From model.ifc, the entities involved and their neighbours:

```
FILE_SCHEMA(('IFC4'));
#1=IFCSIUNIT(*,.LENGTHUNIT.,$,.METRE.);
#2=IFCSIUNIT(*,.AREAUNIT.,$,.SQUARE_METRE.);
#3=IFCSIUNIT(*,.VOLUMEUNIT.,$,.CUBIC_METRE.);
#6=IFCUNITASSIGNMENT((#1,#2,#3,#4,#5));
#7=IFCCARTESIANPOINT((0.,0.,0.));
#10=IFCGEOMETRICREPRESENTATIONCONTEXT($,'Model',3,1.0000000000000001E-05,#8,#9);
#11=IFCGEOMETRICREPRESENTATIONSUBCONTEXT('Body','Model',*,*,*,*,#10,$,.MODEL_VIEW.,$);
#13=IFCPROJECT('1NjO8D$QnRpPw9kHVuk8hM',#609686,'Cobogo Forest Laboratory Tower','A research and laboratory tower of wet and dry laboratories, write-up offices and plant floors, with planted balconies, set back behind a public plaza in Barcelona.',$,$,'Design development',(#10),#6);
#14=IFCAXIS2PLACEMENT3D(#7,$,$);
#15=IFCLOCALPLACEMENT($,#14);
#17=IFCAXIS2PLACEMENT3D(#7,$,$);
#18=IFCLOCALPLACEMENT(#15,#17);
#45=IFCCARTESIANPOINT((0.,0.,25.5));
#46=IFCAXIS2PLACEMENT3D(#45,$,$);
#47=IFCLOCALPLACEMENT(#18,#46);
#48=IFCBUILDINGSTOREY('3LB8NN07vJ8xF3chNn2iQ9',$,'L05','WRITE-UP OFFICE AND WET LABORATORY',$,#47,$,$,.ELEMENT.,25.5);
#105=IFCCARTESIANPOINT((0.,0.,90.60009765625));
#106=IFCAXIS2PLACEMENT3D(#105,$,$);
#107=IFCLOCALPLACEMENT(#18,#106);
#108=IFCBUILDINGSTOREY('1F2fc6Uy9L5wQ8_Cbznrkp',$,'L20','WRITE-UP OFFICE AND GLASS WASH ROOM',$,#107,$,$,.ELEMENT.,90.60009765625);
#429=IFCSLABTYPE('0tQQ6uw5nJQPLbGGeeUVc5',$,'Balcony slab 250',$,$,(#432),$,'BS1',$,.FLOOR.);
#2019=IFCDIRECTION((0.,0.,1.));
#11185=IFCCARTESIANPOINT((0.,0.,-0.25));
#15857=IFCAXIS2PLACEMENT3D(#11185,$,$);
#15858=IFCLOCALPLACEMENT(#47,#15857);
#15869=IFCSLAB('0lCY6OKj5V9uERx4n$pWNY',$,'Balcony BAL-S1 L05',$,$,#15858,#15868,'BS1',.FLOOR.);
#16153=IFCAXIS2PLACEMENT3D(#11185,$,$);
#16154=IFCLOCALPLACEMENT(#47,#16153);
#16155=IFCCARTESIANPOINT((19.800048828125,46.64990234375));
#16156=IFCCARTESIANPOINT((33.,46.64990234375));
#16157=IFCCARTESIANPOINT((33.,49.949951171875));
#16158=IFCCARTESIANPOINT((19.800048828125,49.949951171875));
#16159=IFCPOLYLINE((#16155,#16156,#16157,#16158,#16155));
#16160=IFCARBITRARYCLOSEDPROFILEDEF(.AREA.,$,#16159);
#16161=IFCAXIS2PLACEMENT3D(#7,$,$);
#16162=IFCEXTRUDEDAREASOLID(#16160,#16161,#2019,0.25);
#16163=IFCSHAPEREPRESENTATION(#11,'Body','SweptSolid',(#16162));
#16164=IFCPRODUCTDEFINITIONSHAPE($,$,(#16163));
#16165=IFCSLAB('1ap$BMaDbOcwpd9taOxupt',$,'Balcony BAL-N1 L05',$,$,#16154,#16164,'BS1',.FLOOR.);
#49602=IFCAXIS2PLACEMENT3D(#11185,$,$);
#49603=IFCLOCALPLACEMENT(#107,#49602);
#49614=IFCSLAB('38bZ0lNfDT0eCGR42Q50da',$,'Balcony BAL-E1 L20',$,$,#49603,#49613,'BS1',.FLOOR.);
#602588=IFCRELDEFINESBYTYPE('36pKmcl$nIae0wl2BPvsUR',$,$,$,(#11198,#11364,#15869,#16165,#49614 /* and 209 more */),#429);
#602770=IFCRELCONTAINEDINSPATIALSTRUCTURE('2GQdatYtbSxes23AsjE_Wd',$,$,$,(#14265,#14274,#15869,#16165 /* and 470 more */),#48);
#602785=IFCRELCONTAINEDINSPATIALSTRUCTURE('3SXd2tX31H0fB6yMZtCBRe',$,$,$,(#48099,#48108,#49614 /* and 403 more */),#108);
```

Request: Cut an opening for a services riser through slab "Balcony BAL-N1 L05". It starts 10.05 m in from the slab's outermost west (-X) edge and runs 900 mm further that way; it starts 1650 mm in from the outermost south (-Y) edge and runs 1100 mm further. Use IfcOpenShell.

```python
import numpy as np
import ifcopenshell
import ifcopenshell.api.feature
import ifcopenshell.api.geometry
import ifcopenshell.api.root
import ifcopenshell.geom
import ifcopenshell.util.placement
import ifcopenshell.util.representation
import ifcopenshell.util.shape
import ifcopenshell.util.unit

model = ifcopenshell.open("model.ifc")
unit_scale = ifcopenshell.util.unit.calculate_unit_scale(model)
settings = ifcopenshell.geom.settings()


def volume(element):
    """Net volume in cubic metres, openings subtracted."""
    shape = ifcopenshell.geom.create_shape(settings, element)
    return ifcopenshell.util.shape.get_volume(shape.geometry)


slab = model.by_guid("1ap$BMaDbOcwpd9taOxupt")
before = volume(slab)

# Extent in the slab's own axes, in metres. The edges named are its -X and -Y sides.
slab_shape = ifcopenshell.geom.create_shape(settings, slab)
vertices = ifcopenshell.util.shape.get_vertices(slab_shape.geometry)
x_min, y_min, bottom = vertices.min(axis=0)
top = vertices[:, 2].max()

opening = ifcopenshell.api.root.create_entity(model, ifc_class="IfcOpeningElement", name="Services riser opening", predefined_type="OPENING")
context = ifcopenshell.util.representation.get_context(model, "Model", "Body", "MODEL_VIEW")
width, depth = 0.9, 1.1
outline = [(0.0, 0.0), (width, 0.0), (width, depth), (0.0, depth), (0.0, 0.0)]
# Overshoot both faces by 50 mm so the cut is clean.
shape = ifcopenshell.api.geometry.add_slab_representation(
    model, context=context, depth=top - bottom + 0.1, polyline=outline
)
ifcopenshell.api.geometry.assign_representation(model, product=opening, representation=shape)

matrix = ifcopenshell.util.placement.get_local_placement(slab.ObjectPlacement)
matrix[:, 3] = matrix @ np.append(np.array([x_min + 10.05, y_min + 1.65, bottom - 0.05]) / unit_scale, 1.0)
ifcopenshell.api.geometry.edit_object_placement(model, product=opening, matrix=matrix, is_si=False)
ifcopenshell.api.feature.add_feature(model, feature=opening, element=slab)

after = volume(slab)

print(f"slab volume {before:.3f} -> {after:.3f} m3")

model.write("model_v2.ifc")
```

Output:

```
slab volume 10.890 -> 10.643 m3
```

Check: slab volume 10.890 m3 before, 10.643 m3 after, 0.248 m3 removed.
